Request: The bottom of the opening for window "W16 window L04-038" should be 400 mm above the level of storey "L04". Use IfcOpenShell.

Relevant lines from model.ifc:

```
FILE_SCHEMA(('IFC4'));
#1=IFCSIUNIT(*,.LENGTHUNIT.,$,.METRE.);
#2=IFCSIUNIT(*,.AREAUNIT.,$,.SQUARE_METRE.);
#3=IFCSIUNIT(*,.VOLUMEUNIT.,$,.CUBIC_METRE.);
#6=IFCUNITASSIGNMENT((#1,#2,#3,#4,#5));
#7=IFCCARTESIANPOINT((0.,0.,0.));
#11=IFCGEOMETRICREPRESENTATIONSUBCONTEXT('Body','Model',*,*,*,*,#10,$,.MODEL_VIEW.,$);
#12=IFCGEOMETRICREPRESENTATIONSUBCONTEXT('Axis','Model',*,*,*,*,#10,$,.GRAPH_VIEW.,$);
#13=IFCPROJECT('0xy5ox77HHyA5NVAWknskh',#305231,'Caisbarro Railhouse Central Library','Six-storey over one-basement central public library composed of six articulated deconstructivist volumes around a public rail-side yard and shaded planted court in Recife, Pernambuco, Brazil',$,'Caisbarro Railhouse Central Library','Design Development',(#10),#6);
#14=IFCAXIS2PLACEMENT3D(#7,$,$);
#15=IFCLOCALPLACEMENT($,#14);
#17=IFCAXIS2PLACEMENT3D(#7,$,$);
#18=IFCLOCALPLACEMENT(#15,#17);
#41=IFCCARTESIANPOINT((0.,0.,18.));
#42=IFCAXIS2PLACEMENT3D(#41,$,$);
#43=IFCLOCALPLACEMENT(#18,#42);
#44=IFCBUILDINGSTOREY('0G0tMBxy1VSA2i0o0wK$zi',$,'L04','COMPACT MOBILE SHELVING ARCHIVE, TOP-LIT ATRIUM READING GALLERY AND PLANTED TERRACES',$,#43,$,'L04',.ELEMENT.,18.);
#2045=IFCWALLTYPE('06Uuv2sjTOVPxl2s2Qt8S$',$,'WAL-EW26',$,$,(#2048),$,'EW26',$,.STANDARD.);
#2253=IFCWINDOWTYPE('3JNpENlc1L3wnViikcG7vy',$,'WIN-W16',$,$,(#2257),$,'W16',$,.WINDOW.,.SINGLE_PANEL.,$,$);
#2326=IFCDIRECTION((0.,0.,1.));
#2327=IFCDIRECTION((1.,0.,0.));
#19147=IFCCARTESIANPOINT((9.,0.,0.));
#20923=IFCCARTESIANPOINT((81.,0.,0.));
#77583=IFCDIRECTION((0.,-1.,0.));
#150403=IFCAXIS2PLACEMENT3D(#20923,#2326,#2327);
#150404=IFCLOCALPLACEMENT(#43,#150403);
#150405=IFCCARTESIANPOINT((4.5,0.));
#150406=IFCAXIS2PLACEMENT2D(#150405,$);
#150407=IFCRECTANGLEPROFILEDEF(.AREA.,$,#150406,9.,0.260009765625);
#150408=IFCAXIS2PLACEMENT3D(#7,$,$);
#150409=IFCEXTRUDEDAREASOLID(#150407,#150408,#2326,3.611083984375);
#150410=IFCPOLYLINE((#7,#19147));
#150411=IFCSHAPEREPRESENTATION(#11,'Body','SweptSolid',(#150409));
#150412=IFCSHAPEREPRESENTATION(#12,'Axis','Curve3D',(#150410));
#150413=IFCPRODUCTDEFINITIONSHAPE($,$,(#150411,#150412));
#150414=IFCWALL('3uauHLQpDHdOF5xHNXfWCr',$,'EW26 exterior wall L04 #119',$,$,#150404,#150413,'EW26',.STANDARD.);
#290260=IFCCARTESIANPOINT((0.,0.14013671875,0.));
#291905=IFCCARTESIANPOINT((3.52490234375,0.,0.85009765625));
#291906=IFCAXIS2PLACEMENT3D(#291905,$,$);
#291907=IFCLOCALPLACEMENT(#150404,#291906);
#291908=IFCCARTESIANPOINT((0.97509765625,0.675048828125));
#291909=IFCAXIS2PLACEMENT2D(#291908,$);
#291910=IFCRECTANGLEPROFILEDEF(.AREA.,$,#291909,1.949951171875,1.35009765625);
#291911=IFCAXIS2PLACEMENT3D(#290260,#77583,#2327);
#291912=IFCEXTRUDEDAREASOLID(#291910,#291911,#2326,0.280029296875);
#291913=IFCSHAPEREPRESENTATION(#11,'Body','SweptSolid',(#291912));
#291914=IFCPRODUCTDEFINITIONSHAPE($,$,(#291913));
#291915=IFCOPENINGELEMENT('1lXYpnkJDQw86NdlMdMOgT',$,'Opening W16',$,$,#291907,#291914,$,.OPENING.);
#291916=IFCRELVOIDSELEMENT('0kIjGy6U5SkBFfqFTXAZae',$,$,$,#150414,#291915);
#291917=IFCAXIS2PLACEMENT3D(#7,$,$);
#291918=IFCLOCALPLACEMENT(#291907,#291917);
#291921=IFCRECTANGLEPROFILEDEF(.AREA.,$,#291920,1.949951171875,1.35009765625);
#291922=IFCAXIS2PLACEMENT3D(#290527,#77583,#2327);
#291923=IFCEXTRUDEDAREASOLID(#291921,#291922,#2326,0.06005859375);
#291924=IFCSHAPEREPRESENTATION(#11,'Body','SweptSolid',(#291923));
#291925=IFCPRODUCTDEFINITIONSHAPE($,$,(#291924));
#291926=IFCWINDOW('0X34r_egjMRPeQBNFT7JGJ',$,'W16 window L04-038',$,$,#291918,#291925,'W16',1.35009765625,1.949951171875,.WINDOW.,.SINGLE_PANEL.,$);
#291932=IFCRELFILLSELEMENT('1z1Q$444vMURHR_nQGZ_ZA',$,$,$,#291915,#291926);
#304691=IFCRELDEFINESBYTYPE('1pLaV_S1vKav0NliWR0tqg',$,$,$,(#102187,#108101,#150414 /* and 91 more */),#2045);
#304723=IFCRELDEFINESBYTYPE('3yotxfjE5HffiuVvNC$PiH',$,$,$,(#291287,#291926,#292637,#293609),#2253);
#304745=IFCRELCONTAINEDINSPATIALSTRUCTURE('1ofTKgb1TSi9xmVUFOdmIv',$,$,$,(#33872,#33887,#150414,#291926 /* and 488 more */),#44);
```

```python
import numpy as np
import ifcopenshell
import ifcopenshell.api.geometry
import ifcopenshell.geom
import ifcopenshell.util.element
import ifcopenshell.util.placement
import ifcopenshell.util.shape
import ifcopenshell.util.unit

model = ifcopenshell.open("model.ifc")
unit_scale = ifcopenshell.util.unit.calculate_unit_scale(model)

window = model.by_id(291926)
opening = window.FillsVoids[0].RelatingOpeningElement
storey = ifcopenshell.util.element.get_container(window, ifc_class="IfcBuildingStorey")
level = ifcopenshell.util.placement.get_local_placement(storey.ObjectPlacement)[2, 3]

# The opening's origin need not be at the sill, so measure its lowest point.
shape = ifcopenshell.geom.create_shape(ifcopenshell.geom.settings(), opening)
bottom = ifcopenshell.util.shape.get_shape_bottom_elevation(shape, shape.geometry) / unit_scale
dz = level + 0.4 - bottom

shift = np.array([0.0, 0.0, dz])
# The window is placed relative to its opening, so it follows when the opening moves.
matrix = ifcopenshell.util.placement.get_local_placement(opening.ObjectPlacement)
matrix[:3, 3] += shift
ifcopenshell.api.geometry.edit_object_placement(
    model, product=opening, matrix=matrix, is_si=False, should_transform_children=True
)

print(f"moved by {dz * unit_scale:+.3f} m")

model.write("model_edited.ifc")
```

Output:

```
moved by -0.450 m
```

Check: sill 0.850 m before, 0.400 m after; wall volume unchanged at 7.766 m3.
